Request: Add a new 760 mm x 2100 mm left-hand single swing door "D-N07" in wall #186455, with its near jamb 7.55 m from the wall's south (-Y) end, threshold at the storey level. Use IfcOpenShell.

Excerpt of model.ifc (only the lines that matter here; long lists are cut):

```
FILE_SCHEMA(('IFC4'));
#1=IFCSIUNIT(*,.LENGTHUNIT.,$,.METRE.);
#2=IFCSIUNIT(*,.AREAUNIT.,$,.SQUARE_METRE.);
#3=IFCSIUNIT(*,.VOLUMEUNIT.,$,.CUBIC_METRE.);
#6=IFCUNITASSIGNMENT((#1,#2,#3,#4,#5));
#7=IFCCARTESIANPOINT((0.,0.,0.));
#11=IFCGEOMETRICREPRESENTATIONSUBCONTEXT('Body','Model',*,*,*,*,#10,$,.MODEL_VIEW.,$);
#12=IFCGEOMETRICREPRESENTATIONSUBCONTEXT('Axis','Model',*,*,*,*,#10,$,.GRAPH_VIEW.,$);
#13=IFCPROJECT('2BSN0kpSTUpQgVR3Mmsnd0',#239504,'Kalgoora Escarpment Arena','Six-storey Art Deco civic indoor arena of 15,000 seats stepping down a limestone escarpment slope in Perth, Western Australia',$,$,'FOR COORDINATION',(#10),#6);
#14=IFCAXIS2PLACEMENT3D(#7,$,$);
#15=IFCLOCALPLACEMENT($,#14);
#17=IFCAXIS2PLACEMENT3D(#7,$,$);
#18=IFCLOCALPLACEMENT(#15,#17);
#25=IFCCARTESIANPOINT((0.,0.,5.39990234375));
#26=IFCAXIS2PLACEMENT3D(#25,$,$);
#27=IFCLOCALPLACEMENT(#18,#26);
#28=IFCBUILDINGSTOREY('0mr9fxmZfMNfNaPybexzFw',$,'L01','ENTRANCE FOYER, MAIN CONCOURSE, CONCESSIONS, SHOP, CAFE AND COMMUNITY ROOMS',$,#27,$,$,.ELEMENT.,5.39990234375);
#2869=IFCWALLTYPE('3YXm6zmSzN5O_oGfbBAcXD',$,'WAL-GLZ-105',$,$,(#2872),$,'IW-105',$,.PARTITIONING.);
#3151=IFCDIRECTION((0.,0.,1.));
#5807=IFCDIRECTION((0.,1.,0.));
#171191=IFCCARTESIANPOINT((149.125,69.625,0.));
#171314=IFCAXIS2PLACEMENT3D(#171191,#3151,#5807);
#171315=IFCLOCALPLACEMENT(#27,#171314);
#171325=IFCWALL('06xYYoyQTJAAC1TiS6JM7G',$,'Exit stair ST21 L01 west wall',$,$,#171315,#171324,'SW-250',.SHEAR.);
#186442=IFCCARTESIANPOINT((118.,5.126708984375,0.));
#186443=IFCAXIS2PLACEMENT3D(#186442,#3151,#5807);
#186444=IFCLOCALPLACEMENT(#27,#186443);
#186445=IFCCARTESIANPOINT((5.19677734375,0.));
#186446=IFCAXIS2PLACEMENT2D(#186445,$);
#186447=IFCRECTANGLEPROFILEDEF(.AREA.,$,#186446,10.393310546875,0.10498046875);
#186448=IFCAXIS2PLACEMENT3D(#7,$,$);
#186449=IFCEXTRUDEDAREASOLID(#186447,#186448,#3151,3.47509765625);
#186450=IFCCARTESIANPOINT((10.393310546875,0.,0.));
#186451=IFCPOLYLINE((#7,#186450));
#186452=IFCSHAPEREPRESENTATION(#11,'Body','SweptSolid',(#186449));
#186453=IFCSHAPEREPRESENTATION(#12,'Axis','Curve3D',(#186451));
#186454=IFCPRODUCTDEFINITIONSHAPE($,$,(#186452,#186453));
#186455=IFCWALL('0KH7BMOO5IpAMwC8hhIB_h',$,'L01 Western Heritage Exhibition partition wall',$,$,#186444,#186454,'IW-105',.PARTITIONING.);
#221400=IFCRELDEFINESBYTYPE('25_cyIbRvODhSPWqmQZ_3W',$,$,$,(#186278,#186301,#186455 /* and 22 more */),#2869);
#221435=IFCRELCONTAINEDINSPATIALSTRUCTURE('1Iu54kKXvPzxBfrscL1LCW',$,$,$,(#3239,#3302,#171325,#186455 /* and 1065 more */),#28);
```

```python
import numpy as np
import ifcopenshell
import ifcopenshell.api.feature
import ifcopenshell.api.geometry
import ifcopenshell.api.root
import ifcopenshell.api.spatial
import ifcopenshell.geom
import ifcopenshell.util.element
import ifcopenshell.util.placement
import ifcopenshell.util.representation
import ifcopenshell.util.shape
import ifcopenshell.util.unit

model = ifcopenshell.open("model.ifc")
unit_scale = ifcopenshell.util.unit.calculate_unit_scale(model)
settings = ifcopenshell.geom.settings()


def volume(element):
    """Net volume in cubic metres, openings subtracted."""
    shape = ifcopenshell.geom.create_shape(settings, element)
    return ifcopenshell.util.shape.get_volume(shape.geometry)


wall = model.by_id(186455)
storey = ifcopenshell.util.element.get_container(wall, ifc_class="IfcBuildingStorey")
context = ifcopenshell.util.representation.get_context(model, "Model", "Body", "MODEL_VIEW")
before = volume(wall)

width, height, from_end, sill = 0.76, 2.1, 7.55, 0.0  # metres

# The wall runs along its own X axis, and the end named is its -X end.
wall_shape = ifcopenshell.geom.create_shape(settings, wall)
x, y, z = ifcopenshell.util.shape.get_vertices(wall_shape.geometry).T
start = x.min() + from_end
face, thickness = float(y.min()), float(y.max() - y.min())
wall_matrix = ifcopenshell.util.placement.get_local_placement(wall.ObjectPlacement)
level = ifcopenshell.util.placement.get_local_placement(storey.ObjectPlacement)[2, 3]


def in_wall(x, y):
    """Placement at x, y metres in the wall's axes, at sill height."""
    matrix = wall_matrix.copy()
    matrix[:, 3] = wall_matrix @ np.array([x / unit_scale, y / unit_scale, 0.0, 1.0])
    matrix[2, 3] = level + sill / unit_scale
    return matrix


# Opening: a box that overshoots both wall faces by 50 mm.
opening = ifcopenshell.api.root.create_entity(model, ifc_class="IfcOpeningElement", predefined_type="OPENING")
box = ifcopenshell.api.geometry.add_wall_representation(
    model, context=context, length=width, height=height, thickness=thickness + 0.1
)
ifcopenshell.api.geometry.assign_representation(model, product=opening, representation=box)
ifcopenshell.api.geometry.edit_object_placement(model, product=opening, matrix=in_wall(start, face - 0.05), is_si=False)
ifcopenshell.api.feature.add_feature(model, feature=opening, element=wall)

door = ifcopenshell.api.root.create_entity(model, ifc_class="IfcDoor", name="D-N07", predefined_type="DOOR")
door.OverallWidth, door.OverallHeight = width / unit_scale, height / unit_scale
door.OperationType = "SINGLE_SWING_LEFT"
body = ifcopenshell.api.geometry.add_door_representation(
    model,
    context=context,
    overall_width=door.OverallWidth,
    overall_height=door.OverallHeight,
    operation_type="SINGLE_SWING_LEFT",
    lining_properties={"LiningDepth": thickness / unit_scale, "ThresholdDepth": thickness / unit_scale},
)
ifcopenshell.api.geometry.assign_representation(model, product=door, representation=body)
ifcopenshell.api.spatial.assign_container(model, products=[door], relating_structure=storey)
ifcopenshell.api.feature.add_filling(model, opening=opening, element=door)

# The lining spans the wall, so the door starts at the wall face.
ifcopenshell.api.geometry.edit_object_placement(model, product=door, matrix=in_wall(start, face), is_si=False)

after = volume(wall)

print(f"wall volume {before:.3f} -> {after:.3f} m3")

model.write("model_edited.ifc")
```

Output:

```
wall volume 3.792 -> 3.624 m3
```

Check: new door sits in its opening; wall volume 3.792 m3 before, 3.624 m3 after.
